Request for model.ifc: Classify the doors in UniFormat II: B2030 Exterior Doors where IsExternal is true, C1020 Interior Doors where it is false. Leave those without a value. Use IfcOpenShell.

First a look at what the model holds.

```python
import ifcopenshell
import ifcopenshell.util.element

model = ifcopenshell.open("model.ifc")
print(model.schema)
print("classifications:", [c.Name for c in model.by_type("IfcClassification")])
values = [ifcopenshell.util.element.get_pset(e, "Pset_DoorCommon", "IsExternal") for e in model.by_type("IfcDoor")]
for value in (True, False, None):
    print("IsExternal", value, values.count(value))
```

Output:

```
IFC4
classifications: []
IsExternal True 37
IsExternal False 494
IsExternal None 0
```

```python
import ifcopenshell
import ifcopenshell.api.classification
import ifcopenshell.util.element

model = ifcopenshell.open("model.ifc")

system = ifcopenshell.api.classification.add_classification(model, classification="UniFormat II")

doors = model.by_type("IfcDoor")
external = {e: ifcopenshell.util.element.get_pset(e, "Pset_DoorCommon", "IsExternal") for e in doors}
for flag, code, name in ((True, "B2030", "Exterior Doors"), (False, "C1020", "Interior Doors")):
    products = [e for e in doors if external[e] is flag]
    ifcopenshell.api.classification.add_reference(
        model, products=products, classification=system, identification=code, name=name
    )
    print(code, len(products))

model.write("model_v2.ifc")
```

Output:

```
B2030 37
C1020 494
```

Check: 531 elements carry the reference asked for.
